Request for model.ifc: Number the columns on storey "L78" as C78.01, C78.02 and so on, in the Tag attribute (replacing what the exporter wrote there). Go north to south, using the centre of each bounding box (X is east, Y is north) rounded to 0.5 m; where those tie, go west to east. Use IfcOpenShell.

First a look at what the model holds.

```python
import ifcopenshell
import ifcopenshell.util.element
import ifcopenshell.util.placement

model = ifcopenshell.open("model.ifc")
print(model.schema)
storey = next(s for s in model.by_type("IfcBuildingStorey") if s.Name == "L78")
columns = [e for e in ifcopenshell.util.element.get_decomposition(storey) if e.is_a("IfcColumn")]
for e in sorted(columns, key=lambda e: e.id()):
    origin = ifcopenshell.util.placement.get_local_placement(e.ObjectPlacement)[:3, 3]
    print(e.id(), e.Tag, e.Name, origin.round(2) + 0.0, sep=" | ")
```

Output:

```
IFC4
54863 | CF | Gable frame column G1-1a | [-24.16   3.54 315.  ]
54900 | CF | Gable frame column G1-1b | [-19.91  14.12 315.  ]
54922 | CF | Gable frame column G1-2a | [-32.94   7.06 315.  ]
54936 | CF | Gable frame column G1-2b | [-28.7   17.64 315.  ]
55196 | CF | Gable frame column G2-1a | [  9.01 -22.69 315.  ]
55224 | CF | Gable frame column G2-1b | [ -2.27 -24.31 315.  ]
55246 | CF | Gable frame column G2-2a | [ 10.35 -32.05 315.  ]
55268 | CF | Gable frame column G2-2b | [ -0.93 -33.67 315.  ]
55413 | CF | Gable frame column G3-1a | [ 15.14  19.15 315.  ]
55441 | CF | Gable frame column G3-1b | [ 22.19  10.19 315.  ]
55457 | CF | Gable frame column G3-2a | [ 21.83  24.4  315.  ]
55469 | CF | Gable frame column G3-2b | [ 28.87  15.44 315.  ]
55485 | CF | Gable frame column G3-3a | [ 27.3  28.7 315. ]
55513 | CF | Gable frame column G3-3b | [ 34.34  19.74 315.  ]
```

```python
import ifcopenshell
import ifcopenshell.geom
import ifcopenshell.util.element
import ifcopenshell.util.shape

model = ifcopenshell.open("model.ifc")
settings = ifcopenshell.geom.settings()
settings.set("use-world-coords", True)


def centre(element):
    shape = ifcopenshell.geom.create_shape(settings, element)
    return ifcopenshell.util.shape.get_bbox_centroid(shape.geometry)


storey = next(s for s in model.by_type("IfcBuildingStorey") if s.Name == "L78")
columns = [e for e in ifcopenshell.util.element.get_decomposition(storey) if e.is_a("IfcColumn")]

# Insertion points can sit at a corner or the storey origin, so sort by the geometry (in metres).
centres = {e: centre(e) for e in columns}
columns.sort(key=lambda e: (-round(centres[e][1] / 0.5), centres[e][0]))

for i, e in enumerate(columns, start=1):
    number = f"C78.{i:02d}"
    e.Tag = number
    print(e.id(), number)

model.write("model_rev.ifc")
```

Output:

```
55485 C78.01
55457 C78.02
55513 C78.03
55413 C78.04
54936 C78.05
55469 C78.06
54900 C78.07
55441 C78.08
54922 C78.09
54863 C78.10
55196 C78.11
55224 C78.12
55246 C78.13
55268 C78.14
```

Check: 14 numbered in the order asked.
